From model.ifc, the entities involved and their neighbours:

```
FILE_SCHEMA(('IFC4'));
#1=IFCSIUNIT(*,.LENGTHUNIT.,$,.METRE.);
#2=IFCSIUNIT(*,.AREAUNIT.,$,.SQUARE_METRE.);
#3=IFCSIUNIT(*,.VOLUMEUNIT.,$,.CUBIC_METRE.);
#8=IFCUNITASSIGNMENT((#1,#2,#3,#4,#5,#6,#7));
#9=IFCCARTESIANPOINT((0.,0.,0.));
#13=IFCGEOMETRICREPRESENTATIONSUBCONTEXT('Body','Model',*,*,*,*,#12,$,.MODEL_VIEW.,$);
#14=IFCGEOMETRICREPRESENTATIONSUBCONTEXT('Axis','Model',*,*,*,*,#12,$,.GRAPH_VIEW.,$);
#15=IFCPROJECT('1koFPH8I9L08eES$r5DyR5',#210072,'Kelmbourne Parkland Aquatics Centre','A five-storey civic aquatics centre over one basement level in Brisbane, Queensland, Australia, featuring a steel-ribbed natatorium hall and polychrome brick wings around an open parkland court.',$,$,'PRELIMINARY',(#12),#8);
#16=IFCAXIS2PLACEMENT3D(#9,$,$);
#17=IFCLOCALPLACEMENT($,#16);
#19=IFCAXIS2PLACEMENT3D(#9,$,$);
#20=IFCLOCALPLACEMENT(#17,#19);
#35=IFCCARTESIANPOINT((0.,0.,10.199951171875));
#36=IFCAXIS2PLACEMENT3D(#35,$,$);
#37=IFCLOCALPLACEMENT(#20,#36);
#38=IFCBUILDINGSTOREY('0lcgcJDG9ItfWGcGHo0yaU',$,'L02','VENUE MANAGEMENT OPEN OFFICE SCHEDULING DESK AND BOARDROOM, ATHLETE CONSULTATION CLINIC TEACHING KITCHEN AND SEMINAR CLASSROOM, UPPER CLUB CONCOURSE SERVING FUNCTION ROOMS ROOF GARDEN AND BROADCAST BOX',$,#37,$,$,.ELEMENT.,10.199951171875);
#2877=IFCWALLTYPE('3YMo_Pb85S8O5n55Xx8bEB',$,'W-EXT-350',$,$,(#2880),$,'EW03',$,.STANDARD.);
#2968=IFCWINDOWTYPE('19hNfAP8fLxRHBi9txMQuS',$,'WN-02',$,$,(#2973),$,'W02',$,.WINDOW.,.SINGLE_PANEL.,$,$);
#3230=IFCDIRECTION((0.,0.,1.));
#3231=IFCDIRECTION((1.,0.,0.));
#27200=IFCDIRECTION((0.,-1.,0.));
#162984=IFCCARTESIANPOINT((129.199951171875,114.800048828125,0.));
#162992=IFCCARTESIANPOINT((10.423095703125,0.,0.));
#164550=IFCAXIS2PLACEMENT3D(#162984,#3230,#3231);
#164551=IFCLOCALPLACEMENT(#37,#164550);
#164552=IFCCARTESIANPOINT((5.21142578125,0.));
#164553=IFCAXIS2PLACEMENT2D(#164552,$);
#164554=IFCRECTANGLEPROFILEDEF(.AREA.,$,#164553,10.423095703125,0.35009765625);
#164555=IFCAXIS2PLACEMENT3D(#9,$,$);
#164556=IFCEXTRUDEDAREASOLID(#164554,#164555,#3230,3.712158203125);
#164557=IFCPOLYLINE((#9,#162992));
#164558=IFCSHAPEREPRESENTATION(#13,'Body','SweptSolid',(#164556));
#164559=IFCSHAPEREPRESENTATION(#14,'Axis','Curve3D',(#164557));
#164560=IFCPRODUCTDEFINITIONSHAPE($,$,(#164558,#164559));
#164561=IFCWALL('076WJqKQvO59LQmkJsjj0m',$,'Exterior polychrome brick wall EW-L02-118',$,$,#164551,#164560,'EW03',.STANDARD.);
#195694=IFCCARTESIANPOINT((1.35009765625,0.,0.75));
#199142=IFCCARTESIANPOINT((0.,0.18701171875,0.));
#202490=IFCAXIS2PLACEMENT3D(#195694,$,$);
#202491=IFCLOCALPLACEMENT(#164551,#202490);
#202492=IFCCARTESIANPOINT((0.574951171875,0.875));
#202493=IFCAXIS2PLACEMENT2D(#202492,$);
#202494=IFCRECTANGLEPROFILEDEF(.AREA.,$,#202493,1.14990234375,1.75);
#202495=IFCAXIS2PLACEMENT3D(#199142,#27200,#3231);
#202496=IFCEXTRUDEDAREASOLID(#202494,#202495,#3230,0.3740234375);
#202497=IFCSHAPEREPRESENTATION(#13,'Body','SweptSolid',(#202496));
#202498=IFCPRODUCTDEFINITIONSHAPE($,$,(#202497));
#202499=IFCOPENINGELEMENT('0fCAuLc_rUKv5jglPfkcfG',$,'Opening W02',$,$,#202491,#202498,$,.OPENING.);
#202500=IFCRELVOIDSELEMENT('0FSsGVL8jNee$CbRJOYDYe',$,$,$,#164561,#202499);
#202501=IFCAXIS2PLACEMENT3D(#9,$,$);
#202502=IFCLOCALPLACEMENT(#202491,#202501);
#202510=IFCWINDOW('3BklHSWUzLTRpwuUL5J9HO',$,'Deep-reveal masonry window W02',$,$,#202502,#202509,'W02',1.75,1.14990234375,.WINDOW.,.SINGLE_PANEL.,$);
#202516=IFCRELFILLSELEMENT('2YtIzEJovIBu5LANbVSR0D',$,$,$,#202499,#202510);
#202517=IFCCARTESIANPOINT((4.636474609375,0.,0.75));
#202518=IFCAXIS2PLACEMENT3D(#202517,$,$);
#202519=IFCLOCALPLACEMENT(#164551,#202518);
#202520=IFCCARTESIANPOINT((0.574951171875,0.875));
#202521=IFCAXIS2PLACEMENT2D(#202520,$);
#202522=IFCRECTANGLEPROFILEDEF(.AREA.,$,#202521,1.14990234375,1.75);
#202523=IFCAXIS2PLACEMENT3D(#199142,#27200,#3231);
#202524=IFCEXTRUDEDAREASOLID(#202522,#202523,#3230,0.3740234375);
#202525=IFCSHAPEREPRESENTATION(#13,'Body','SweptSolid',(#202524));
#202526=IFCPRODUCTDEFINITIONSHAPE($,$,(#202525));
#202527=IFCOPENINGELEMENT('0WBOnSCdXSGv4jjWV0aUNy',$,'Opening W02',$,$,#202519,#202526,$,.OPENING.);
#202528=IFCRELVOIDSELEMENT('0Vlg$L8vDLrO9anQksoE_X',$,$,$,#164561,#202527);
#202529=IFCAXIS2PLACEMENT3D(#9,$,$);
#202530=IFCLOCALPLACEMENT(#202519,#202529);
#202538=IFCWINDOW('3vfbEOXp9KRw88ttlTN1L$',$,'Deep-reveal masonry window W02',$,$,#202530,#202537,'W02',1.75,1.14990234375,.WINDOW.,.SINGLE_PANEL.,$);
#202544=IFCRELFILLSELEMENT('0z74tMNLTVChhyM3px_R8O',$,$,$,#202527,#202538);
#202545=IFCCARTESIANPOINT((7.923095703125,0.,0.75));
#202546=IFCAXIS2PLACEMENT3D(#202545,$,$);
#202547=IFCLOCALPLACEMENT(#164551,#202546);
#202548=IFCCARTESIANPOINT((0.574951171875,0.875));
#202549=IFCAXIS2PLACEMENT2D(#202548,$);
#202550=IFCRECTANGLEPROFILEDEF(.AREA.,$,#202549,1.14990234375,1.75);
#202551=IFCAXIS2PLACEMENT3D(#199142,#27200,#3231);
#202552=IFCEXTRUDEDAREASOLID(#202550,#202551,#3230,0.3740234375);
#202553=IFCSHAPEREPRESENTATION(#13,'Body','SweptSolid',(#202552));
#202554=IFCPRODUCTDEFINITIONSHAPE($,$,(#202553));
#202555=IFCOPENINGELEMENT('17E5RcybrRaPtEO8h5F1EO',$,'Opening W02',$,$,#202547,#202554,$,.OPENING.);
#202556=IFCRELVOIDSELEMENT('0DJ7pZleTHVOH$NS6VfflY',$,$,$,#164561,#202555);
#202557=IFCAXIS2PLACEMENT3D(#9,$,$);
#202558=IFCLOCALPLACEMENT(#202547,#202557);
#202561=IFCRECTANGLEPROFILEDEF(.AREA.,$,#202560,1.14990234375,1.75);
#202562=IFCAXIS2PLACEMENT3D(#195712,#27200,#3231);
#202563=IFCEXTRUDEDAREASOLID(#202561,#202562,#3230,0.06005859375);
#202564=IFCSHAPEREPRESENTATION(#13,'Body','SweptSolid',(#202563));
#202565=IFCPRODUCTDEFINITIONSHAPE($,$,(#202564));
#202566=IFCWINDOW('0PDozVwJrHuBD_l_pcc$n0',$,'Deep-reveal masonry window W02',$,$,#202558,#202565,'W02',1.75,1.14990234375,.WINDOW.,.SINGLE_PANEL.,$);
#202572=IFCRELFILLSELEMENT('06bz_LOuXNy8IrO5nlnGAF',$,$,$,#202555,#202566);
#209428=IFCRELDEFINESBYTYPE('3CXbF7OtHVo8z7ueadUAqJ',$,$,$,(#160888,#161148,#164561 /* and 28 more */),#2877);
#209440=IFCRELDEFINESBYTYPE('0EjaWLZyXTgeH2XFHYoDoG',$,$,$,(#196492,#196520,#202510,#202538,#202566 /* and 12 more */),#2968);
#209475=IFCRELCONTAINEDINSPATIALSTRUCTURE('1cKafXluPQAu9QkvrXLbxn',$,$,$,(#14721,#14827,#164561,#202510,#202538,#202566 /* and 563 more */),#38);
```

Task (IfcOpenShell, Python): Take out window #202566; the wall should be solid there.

```python
import ifcopenshell
import ifcopenshell.api.feature
import ifcopenshell.api.root
import ifcopenshell.geom
import ifcopenshell.util.shape

model = ifcopenshell.open("model.ifc")
settings = ifcopenshell.geom.settings()


def volume(element):
    """Net volume in cubic metres, openings subtracted."""
    shape = ifcopenshell.geom.create_shape(settings, element)
    return ifcopenshell.util.shape.get_volume(shape.geometry)


window = model.by_guid("0PDozVwJrHuBD_l_pcc$n0")
opening = window.FillsVoids[0].RelatingOpeningElement
wall = opening.VoidsElements[0].RelatingBuildingElement
before = volume(wall)

ifcopenshell.api.root.remove_product(model, product=window)
ifcopenshell.api.feature.remove_feature(model, feature=opening)

after = volume(wall)

print(f"wall volume {before:.3f} -> {after:.3f} m3")

model.write("model-out.ifc")
```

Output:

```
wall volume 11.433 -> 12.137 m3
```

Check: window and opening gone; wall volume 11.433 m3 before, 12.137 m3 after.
